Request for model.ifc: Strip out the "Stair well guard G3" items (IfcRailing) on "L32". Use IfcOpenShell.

First a look at what the model holds.

```python
import ifcopenshell
import ifcopenshell.util.element

model = ifcopenshell.open("model.ifc")
print(model.schema)
storey = next(s for s in model.by_type("IfcBuildingStorey") if s.Name == "L32")
railings = [e for e in ifcopenshell.util.element.get_decomposition(storey) if e.is_a("IfcRailing")]
seen = {}
for e in railings:
    element_type = ifcopenshell.util.element.get_type(e)
    name = element_type.Name if element_type not in (None, e) else None
    seen[name] = seen.get(name, 0) + 1
for name, count in sorted(seen.items(), key=str):
    print(count, "x", name)
```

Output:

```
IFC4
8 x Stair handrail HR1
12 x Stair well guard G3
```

```python
import ifcopenshell
import ifcopenshell.api.root
import ifcopenshell.util.element

model = ifcopenshell.open("model.ifc")

storey = next(s for s in model.by_type("IfcBuildingStorey") if s.Name == "L32")
railings = [e for e in ifcopenshell.util.element.get_decomposition(storey) if e.is_a("IfcRailing")]
targets = [e for e in railings if (t := ifcopenshell.util.element.get_type(e)) not in (None, e) and t.Name == "Stair well guard G3"]

for e in targets:
    ifcopenshell.api.root.remove_product(model, product=e)
print(len(targets), "removed")

model.write("model_updated.ifc")
```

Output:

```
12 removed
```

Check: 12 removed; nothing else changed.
